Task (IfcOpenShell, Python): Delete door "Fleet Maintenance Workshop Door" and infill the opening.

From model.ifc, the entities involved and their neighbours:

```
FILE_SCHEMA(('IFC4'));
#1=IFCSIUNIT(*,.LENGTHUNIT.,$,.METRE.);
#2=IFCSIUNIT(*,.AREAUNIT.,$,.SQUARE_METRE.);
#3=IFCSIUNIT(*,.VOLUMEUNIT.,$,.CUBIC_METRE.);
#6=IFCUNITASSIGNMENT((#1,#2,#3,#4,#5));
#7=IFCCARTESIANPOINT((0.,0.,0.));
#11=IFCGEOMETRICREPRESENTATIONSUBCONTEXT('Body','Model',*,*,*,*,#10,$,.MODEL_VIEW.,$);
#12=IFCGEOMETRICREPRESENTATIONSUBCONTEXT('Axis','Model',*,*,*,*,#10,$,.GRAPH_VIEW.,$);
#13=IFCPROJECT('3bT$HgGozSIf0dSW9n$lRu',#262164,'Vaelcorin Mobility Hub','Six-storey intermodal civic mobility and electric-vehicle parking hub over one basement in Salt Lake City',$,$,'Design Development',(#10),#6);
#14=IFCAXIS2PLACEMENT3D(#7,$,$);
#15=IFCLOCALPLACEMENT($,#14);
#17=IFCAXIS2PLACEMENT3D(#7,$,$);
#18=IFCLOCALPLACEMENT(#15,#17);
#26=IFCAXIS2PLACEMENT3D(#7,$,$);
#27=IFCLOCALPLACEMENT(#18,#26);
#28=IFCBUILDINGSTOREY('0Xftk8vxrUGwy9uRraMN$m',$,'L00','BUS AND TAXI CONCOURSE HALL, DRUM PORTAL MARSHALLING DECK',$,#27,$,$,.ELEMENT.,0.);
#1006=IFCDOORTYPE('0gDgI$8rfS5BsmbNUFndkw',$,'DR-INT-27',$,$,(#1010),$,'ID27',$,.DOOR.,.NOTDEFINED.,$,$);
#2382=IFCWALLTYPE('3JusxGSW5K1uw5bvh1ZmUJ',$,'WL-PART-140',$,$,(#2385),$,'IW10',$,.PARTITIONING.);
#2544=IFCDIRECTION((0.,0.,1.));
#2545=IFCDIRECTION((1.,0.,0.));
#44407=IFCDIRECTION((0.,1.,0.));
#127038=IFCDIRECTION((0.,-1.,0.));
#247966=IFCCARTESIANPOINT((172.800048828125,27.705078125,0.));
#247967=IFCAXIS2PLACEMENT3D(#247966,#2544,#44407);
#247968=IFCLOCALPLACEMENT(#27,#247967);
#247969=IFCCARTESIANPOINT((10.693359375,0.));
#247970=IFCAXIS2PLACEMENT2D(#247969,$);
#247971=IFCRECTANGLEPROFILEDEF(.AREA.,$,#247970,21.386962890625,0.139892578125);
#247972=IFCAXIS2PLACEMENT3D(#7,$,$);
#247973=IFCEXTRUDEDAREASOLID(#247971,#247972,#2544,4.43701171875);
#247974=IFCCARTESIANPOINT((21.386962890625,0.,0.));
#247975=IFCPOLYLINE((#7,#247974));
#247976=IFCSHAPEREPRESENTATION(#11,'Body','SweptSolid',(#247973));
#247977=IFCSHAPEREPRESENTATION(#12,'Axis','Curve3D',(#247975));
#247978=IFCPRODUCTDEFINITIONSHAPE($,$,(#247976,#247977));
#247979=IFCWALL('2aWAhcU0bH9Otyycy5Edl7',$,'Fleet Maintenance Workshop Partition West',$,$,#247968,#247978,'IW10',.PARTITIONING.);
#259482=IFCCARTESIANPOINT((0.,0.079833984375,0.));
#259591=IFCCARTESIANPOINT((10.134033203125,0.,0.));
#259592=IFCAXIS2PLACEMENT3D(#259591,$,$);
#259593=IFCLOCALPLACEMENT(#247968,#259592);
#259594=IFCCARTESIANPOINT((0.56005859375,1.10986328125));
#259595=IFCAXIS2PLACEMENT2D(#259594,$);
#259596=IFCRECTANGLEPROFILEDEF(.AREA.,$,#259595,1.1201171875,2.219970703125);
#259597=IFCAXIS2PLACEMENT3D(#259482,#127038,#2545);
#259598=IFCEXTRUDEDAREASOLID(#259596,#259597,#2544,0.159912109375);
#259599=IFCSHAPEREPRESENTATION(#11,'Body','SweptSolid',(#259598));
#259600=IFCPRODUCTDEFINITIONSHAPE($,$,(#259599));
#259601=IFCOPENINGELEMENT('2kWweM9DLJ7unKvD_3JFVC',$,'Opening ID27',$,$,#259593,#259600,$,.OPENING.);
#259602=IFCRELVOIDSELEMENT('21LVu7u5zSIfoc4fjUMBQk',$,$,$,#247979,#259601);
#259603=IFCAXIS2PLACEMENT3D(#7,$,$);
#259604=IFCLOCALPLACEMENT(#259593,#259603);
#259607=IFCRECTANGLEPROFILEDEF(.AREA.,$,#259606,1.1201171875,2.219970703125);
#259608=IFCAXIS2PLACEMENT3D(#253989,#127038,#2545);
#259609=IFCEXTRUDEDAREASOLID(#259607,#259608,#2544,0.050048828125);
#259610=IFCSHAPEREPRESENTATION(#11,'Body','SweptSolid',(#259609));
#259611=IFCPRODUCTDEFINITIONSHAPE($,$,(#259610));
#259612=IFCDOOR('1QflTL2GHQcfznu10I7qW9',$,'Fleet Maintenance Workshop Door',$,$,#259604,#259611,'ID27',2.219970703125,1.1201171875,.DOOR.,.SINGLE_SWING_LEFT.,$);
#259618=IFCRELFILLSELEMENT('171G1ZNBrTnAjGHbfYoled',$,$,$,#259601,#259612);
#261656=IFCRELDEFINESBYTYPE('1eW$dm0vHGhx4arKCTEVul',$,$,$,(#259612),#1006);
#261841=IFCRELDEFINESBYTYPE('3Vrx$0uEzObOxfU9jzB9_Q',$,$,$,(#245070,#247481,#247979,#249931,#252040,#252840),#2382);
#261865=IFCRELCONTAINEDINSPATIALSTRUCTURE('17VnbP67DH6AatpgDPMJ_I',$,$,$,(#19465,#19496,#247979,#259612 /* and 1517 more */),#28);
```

```python
import ifcopenshell
import ifcopenshell.api.feature
import ifcopenshell.api.root
import ifcopenshell.geom
import ifcopenshell.util.shape

model = ifcopenshell.open("model.ifc")
settings = ifcopenshell.geom.settings()


def volume(element):
    """Net volume in cubic metres, openings subtracted."""
    shape = ifcopenshell.geom.create_shape(settings, element)
    return ifcopenshell.util.shape.get_volume(shape.geometry)


door = model.by_guid("1QflTL2GHQcfznu10I7qW9")
opening = door.FillsVoids[0].RelatingOpeningElement
wall = opening.VoidsElements[0].RelatingBuildingElement
before = volume(wall)

ifcopenshell.api.root.remove_product(model, product=door)
ifcopenshell.api.feature.remove_feature(model, feature=opening)

after = volume(wall)

print(f"wall volume {before:.3f} -> {after:.3f} m3")

model.write("model_rev.ifc")
```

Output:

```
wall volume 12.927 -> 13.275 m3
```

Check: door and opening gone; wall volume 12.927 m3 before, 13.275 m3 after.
